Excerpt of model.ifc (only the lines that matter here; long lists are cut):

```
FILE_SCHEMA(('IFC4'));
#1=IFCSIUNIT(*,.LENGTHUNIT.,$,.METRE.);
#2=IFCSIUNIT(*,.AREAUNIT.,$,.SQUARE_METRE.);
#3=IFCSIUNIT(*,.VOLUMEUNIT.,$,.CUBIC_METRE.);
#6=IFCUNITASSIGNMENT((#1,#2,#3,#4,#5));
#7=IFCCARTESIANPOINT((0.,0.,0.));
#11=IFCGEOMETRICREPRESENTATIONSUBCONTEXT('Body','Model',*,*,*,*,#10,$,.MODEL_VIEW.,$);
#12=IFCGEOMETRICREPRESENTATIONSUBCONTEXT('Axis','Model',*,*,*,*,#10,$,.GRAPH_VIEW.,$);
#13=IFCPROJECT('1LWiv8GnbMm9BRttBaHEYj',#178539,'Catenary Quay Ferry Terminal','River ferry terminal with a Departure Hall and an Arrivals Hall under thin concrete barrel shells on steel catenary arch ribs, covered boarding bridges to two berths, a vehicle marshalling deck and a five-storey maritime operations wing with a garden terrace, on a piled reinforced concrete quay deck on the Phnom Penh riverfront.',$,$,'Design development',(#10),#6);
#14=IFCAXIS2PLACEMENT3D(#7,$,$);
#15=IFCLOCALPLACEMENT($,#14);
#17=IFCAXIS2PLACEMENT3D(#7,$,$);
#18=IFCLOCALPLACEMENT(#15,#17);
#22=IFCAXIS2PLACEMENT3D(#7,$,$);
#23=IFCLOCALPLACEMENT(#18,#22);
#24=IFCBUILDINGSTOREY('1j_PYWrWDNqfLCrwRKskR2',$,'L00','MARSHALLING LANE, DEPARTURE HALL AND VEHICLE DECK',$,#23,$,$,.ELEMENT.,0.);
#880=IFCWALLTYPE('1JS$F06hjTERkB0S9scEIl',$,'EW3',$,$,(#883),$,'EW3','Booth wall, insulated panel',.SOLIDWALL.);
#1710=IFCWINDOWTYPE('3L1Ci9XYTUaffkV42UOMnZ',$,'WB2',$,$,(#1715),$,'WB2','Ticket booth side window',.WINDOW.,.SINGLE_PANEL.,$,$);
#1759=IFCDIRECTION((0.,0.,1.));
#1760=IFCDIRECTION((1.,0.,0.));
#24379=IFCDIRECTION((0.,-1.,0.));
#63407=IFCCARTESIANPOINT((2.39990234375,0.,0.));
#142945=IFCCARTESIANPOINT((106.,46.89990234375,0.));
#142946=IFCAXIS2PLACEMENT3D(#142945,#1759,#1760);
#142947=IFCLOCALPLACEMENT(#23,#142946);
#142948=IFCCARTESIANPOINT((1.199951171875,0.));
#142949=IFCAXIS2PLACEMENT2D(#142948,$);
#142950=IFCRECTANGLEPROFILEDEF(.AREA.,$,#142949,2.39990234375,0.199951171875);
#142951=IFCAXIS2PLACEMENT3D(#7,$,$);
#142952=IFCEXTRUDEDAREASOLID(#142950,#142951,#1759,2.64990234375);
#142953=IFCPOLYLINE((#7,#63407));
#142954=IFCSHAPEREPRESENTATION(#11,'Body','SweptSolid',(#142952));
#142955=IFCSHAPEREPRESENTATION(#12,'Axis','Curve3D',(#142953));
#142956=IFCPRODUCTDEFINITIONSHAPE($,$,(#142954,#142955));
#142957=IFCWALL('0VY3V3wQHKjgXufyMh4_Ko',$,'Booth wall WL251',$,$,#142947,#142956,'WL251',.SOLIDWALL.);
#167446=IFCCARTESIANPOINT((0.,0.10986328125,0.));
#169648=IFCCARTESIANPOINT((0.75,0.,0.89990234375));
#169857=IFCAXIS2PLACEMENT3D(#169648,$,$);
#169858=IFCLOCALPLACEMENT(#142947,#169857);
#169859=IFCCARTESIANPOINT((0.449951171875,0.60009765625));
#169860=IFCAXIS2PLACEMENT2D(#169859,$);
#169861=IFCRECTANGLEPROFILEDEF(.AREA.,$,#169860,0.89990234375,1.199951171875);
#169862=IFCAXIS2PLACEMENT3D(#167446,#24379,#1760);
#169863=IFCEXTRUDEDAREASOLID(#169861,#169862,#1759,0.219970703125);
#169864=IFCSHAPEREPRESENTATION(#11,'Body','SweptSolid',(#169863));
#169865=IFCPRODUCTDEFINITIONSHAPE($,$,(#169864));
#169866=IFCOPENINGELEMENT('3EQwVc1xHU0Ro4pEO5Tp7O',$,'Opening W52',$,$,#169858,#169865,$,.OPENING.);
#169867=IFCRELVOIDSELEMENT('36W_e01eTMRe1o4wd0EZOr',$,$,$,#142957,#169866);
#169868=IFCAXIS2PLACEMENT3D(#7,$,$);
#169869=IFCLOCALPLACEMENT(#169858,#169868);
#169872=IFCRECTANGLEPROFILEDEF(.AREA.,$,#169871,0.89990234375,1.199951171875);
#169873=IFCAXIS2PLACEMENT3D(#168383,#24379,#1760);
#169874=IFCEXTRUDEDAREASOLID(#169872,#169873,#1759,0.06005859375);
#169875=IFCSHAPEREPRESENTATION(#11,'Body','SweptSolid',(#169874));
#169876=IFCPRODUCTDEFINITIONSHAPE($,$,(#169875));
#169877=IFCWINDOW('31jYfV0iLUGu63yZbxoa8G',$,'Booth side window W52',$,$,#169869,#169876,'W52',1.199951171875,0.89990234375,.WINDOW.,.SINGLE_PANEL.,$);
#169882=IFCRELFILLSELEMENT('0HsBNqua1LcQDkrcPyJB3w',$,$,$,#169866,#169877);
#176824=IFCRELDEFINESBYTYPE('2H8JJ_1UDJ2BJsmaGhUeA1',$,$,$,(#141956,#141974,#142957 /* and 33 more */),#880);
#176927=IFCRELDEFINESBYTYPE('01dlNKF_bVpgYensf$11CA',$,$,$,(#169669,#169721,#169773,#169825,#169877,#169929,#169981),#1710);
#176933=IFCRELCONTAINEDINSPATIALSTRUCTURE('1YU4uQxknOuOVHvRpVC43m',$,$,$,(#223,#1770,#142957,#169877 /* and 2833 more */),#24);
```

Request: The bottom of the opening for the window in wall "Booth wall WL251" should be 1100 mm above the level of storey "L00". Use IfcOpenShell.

```python
import numpy as np
import ifcopenshell
import ifcopenshell.api.geometry
import ifcopenshell.geom
import ifcopenshell.util.element
import ifcopenshell.util.placement
import ifcopenshell.util.shape
import ifcopenshell.util.unit

model = ifcopenshell.open("model.ifc")
unit_scale = ifcopenshell.util.unit.calculate_unit_scale(model)

window = model.by_guid("31jYfV0iLUGu63yZbxoa8G")
opening = window.FillsVoids[0].RelatingOpeningElement
storey = ifcopenshell.util.element.get_container(window, ifc_class="IfcBuildingStorey")
level = ifcopenshell.util.placement.get_local_placement(storey.ObjectPlacement)[2, 3]

# The opening's origin need not be at the sill, so measure its lowest point.
shape = ifcopenshell.geom.create_shape(ifcopenshell.geom.settings(), opening)
bottom = ifcopenshell.util.shape.get_shape_bottom_elevation(shape, shape.geometry) / unit_scale
dz = level + 1.1 / unit_scale - bottom

shift = np.array([0.0, 0.0, dz])
# The window is placed relative to its opening, so it follows when the opening moves.
matrix = ifcopenshell.util.placement.get_local_placement(opening.ObjectPlacement)
matrix[:3, 3] += shift
ifcopenshell.api.geometry.edit_object_placement(
    model, product=opening, matrix=matrix, is_si=False, should_transform_children=True
)

print(f"moved by {dz * unit_scale:+.3f} m")

model.write("model-out.ifc")
```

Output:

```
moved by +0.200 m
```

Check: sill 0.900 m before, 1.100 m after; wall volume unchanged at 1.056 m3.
